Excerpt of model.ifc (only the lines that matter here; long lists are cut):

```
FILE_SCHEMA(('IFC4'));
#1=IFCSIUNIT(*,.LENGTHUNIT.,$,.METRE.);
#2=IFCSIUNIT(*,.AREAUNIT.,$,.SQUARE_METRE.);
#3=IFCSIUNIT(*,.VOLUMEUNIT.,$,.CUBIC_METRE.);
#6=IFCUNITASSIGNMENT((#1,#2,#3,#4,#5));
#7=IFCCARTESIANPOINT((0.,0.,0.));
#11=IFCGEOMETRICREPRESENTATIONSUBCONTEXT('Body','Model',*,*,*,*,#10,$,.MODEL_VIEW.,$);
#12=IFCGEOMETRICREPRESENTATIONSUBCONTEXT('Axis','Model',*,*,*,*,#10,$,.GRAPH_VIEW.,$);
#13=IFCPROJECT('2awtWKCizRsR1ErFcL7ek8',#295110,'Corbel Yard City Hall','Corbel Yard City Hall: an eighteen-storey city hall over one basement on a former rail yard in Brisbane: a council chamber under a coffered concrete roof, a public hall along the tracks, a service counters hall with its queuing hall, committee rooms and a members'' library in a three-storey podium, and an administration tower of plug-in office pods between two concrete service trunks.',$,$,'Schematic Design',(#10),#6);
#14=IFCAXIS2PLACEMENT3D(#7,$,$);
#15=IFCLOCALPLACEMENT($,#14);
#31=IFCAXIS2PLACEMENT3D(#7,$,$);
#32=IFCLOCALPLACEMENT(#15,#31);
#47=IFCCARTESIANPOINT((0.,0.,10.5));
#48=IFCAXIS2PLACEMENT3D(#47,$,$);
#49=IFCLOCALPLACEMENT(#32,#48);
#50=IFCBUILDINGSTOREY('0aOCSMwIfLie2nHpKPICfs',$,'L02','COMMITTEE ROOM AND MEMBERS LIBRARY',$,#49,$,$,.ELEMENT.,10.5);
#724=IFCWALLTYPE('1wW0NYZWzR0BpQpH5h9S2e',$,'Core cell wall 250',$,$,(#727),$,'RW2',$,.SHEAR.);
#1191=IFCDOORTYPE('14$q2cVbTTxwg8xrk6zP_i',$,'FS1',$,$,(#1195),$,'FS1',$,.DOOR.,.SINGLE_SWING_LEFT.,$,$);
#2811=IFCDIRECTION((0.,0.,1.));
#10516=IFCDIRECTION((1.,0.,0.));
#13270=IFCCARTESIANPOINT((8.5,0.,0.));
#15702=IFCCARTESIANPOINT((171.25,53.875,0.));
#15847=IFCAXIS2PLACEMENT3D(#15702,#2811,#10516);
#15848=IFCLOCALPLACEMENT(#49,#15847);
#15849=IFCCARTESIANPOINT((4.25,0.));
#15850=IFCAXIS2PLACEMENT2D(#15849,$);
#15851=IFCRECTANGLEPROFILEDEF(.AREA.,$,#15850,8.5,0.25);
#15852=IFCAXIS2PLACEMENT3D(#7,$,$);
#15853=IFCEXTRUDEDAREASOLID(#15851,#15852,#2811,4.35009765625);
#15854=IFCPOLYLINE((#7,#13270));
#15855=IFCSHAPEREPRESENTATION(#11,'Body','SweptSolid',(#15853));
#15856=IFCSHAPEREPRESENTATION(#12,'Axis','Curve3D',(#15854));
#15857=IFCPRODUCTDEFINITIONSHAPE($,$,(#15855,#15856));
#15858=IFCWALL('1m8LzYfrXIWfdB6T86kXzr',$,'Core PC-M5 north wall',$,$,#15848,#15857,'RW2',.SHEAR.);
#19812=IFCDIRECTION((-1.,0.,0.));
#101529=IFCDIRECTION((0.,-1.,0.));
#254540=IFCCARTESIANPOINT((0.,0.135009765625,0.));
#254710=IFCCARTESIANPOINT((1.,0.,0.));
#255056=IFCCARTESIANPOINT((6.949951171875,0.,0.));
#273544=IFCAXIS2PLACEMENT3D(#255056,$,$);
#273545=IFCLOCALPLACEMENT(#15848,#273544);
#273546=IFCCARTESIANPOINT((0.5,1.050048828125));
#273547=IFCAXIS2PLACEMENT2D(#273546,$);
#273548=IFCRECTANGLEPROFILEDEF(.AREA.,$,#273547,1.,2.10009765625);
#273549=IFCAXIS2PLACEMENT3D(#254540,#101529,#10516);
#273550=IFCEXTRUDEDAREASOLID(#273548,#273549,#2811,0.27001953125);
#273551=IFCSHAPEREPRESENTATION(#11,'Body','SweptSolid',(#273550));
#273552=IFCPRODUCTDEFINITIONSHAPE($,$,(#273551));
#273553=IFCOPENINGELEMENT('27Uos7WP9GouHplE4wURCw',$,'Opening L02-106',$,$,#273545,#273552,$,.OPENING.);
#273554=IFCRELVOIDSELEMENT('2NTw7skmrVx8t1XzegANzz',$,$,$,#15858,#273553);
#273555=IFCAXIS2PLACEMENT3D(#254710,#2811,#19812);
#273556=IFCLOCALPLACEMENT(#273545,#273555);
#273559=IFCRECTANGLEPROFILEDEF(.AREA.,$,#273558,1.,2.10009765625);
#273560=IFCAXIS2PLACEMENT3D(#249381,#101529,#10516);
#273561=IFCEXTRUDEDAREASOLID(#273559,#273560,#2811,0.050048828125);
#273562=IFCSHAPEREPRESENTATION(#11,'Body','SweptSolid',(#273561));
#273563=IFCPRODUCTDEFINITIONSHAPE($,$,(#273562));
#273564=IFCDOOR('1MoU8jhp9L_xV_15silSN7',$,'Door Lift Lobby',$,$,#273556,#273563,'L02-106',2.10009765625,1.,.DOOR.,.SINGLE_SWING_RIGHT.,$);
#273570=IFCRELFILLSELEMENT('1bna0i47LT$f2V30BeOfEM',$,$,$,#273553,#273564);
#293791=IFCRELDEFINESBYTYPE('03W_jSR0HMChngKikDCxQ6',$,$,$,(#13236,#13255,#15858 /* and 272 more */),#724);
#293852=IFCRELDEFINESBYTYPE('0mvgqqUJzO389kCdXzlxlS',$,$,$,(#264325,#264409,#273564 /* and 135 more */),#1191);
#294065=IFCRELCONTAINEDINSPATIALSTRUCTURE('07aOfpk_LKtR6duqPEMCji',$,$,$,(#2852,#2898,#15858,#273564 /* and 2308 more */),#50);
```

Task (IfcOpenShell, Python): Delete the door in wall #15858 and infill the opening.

```python
import ifcopenshell
import ifcopenshell.api.feature
import ifcopenshell.api.root
import ifcopenshell.geom
import ifcopenshell.util.shape

model = ifcopenshell.open("model.ifc")
settings = ifcopenshell.geom.settings()


def volume(element):
    """Net volume in cubic metres, openings subtracted."""
    shape = ifcopenshell.geom.create_shape(settings, element)
    return ifcopenshell.util.shape.get_volume(shape.geometry)


door = model.by_guid("1MoU8jhp9L_xV_15silSN7")
opening = door.FillsVoids[0].RelatingOpeningElement
wall = opening.VoidsElements[0].RelatingBuildingElement
before = volume(wall)

ifcopenshell.api.root.remove_product(model, product=door)
ifcopenshell.api.feature.remove_feature(model, feature=opening)

after = volume(wall)

print(f"wall volume {before:.3f} -> {after:.3f} m3")

model.write("model_edited.ifc")
```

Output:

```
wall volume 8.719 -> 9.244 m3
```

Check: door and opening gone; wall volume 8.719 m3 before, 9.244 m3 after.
